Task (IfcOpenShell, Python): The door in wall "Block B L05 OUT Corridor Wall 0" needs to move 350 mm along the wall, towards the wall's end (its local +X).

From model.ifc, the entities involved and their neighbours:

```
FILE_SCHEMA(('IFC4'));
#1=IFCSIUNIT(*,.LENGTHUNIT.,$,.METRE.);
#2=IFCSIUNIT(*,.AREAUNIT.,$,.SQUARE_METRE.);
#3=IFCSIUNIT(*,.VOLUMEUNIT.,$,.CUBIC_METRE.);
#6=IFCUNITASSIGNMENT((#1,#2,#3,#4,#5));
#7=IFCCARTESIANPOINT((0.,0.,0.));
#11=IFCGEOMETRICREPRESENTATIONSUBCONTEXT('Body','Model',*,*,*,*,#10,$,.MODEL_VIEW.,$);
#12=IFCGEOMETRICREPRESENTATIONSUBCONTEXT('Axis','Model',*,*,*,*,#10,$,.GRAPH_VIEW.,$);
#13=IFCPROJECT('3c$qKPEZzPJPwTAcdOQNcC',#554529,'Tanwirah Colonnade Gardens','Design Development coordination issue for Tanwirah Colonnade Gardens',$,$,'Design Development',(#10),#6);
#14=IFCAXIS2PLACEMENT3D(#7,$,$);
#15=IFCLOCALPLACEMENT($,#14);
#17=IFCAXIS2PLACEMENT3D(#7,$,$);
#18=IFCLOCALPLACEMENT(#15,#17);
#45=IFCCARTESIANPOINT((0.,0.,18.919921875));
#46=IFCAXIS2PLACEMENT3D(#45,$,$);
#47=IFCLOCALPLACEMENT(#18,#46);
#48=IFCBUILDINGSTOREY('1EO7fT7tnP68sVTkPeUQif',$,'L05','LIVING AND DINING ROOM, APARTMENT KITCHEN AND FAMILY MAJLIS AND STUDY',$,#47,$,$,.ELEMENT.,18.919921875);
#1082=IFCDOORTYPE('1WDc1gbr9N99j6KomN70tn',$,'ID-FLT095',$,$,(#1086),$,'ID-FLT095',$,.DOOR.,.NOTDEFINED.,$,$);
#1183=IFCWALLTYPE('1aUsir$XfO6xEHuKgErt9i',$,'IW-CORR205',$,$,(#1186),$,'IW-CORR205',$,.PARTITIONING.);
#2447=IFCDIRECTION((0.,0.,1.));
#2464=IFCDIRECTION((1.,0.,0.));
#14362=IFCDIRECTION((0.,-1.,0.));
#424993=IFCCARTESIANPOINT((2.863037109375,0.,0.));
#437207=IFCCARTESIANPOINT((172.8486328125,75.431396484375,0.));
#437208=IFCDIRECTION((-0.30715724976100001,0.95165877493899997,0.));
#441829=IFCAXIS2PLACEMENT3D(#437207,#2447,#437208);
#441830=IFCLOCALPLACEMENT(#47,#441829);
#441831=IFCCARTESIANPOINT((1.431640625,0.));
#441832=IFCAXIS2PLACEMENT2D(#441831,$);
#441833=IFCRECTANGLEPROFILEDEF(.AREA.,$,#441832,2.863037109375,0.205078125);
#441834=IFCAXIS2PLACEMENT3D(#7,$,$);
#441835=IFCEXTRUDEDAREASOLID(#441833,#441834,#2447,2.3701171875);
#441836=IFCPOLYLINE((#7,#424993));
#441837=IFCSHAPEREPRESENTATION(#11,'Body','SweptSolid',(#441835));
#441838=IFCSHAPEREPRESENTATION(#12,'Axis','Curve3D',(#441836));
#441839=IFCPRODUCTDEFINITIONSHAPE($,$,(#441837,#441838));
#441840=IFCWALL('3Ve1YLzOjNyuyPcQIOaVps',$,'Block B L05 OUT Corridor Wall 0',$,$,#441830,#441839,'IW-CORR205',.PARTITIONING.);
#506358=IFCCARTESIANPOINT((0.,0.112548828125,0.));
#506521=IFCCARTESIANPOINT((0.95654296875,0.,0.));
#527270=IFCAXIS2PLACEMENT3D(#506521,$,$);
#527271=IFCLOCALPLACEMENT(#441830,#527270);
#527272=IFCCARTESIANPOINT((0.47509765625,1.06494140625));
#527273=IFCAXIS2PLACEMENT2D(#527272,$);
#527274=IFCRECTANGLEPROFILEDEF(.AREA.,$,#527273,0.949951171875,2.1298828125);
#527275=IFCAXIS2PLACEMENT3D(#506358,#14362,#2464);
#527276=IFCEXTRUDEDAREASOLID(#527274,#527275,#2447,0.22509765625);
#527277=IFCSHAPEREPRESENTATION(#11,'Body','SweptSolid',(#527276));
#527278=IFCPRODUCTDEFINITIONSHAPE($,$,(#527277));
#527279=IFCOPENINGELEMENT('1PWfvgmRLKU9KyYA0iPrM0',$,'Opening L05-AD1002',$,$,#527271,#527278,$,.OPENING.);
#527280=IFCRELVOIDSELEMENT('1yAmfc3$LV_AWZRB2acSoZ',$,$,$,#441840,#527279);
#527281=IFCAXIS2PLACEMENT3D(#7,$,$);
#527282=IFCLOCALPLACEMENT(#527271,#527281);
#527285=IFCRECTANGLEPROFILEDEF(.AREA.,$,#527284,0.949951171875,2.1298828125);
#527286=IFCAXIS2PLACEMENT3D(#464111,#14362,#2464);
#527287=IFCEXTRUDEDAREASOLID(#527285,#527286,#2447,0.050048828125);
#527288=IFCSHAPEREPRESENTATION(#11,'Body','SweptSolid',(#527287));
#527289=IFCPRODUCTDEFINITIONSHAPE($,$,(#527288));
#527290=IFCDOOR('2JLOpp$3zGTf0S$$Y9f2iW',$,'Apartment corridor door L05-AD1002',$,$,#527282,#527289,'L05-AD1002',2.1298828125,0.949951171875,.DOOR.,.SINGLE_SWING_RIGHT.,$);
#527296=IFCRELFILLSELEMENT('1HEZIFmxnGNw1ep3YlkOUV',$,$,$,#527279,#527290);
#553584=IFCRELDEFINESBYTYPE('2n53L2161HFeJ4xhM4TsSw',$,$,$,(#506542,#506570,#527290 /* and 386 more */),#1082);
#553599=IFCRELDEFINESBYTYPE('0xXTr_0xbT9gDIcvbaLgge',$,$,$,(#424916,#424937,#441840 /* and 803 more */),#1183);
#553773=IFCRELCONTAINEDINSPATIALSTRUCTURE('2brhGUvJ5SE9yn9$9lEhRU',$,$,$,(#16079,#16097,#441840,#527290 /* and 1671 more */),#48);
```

```python
import ifcopenshell
import ifcopenshell.api.geometry
import ifcopenshell.util.placement

model = ifcopenshell.open("model.ifc")

door = model.by_id(527290)
opening = door.FillsVoids[0].RelatingOpeningElement
wall = opening.VoidsElements[0].RelatingBuildingElement

wall_matrix = ifcopenshell.util.placement.get_local_placement(wall.ObjectPlacement)
shift = wall_matrix[:3, 0] * 0.35
before = ifcopenshell.util.placement.get_local_placement(door.ObjectPlacement)[:3, 3].copy()

# The door is placed relative to its opening, so it follows when the opening moves.
matrix = ifcopenshell.util.placement.get_local_placement(opening.ObjectPlacement)
matrix[:3, 3] += shift
ifcopenshell.api.geometry.edit_object_placement(
    model, product=opening, matrix=matrix, is_si=False, should_transform_children=True
)

after = ifcopenshell.util.placement.get_local_placement(door.ObjectPlacement)[:3, 3]
print("door moved by", (after - before).round(3) + 0.0)

model.write("model_rev.ifc")
```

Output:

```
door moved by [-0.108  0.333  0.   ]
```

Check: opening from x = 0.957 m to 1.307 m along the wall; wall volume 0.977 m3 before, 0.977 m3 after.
